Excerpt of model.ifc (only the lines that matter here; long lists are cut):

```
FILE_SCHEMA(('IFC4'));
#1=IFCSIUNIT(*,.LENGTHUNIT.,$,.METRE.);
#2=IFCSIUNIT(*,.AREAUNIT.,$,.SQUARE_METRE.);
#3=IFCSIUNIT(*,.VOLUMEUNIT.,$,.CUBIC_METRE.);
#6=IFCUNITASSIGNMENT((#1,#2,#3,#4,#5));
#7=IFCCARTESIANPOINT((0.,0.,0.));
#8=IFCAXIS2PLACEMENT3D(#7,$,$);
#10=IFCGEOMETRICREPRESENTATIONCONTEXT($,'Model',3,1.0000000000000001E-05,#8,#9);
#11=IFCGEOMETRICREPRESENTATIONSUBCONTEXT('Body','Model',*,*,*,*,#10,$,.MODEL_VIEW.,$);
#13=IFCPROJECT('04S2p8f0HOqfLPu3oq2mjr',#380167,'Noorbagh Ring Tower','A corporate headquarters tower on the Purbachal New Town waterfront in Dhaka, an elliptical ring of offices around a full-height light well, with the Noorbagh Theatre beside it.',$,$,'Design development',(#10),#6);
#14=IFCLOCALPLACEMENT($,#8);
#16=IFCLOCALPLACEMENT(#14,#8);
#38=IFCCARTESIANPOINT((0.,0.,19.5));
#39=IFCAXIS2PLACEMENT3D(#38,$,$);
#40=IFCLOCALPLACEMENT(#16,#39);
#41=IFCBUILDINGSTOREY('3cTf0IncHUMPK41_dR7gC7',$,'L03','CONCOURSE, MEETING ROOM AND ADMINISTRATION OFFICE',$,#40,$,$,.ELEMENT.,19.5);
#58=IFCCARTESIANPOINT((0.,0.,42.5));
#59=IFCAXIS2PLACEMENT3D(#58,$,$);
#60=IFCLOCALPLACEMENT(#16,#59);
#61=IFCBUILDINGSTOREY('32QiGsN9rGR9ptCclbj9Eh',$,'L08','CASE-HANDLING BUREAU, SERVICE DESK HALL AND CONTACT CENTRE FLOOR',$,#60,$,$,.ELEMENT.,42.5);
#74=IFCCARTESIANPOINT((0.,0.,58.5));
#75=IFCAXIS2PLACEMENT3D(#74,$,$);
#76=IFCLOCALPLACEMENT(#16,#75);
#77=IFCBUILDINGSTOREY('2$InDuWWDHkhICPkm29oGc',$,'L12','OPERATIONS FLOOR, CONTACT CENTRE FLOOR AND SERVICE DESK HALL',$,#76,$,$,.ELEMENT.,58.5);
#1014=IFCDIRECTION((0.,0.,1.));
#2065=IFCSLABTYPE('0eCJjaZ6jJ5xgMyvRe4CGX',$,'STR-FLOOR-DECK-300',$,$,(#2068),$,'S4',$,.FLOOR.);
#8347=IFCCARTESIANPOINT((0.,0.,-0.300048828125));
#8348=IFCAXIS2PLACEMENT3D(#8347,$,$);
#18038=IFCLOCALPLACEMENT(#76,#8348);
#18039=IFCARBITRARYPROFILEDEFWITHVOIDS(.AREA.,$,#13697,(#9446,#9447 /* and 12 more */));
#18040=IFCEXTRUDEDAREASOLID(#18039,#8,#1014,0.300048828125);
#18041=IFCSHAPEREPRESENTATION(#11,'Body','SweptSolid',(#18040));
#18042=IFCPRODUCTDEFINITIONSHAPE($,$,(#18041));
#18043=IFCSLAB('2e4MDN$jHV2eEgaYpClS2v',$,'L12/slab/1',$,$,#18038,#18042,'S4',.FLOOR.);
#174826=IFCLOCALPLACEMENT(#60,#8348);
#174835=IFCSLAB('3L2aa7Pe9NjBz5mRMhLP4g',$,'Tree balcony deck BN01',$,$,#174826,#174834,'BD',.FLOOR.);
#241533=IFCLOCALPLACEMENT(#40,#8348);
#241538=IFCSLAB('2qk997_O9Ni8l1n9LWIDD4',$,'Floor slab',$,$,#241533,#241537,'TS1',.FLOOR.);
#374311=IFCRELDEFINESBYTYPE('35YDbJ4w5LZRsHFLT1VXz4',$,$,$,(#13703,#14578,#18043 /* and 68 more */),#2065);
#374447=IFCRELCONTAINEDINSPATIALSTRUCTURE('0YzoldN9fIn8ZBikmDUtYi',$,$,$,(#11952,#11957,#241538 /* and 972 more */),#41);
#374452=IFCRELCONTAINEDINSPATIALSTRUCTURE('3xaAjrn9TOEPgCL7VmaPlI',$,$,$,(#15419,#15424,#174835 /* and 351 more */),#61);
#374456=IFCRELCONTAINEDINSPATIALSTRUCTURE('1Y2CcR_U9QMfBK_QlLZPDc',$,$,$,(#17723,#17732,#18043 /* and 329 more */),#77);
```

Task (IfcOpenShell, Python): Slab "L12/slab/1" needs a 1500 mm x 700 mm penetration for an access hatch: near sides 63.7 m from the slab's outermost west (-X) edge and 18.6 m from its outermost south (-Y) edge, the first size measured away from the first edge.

```python
import numpy as np
import ifcopenshell
import ifcopenshell.api.feature
import ifcopenshell.api.geometry
import ifcopenshell.api.root
import ifcopenshell.geom
import ifcopenshell.util.placement
import ifcopenshell.util.representation
import ifcopenshell.util.shape
import ifcopenshell.util.unit

model = ifcopenshell.open("model.ifc")
unit_scale = ifcopenshell.util.unit.calculate_unit_scale(model)
settings = ifcopenshell.geom.settings()


def volume(element):
    """Net volume in cubic metres, openings subtracted."""
    shape = ifcopenshell.geom.create_shape(settings, element)
    return ifcopenshell.util.shape.get_volume(shape.geometry)


slab = model.by_id(18043)
before = volume(slab)

# Extent in the slab's own axes, in metres. The edges named are its -X and -Y sides.
slab_shape = ifcopenshell.geom.create_shape(settings, slab)
vertices = ifcopenshell.util.shape.get_vertices(slab_shape.geometry)
x_min, y_min, bottom = vertices.min(axis=0)
top = vertices[:, 2].max()

opening = ifcopenshell.api.root.create_entity(model, ifc_class="IfcOpeningElement", name="Access hatch opening", predefined_type="OPENING")
context = ifcopenshell.util.representation.get_context(model, "Model", "Body", "MODEL_VIEW")
width, depth = 1.5, 0.7
outline = [(0.0, 0.0), (width, 0.0), (width, depth), (0.0, depth), (0.0, 0.0)]
# Overshoot both faces by 50 mm so the cut is clean.
shape = ifcopenshell.api.geometry.add_slab_representation(
    model, context=context, depth=top - bottom + 0.1, polyline=outline
)
ifcopenshell.api.geometry.assign_representation(model, product=opening, representation=shape)

matrix = ifcopenshell.util.placement.get_local_placement(slab.ObjectPlacement)
matrix[:, 3] = matrix @ np.append(np.array([x_min + 63.7, y_min + 18.6, bottom - 0.05]) / unit_scale, 1.0)
ifcopenshell.api.geometry.edit_object_placement(model, product=opening, matrix=matrix, is_si=False)
ifcopenshell.api.feature.add_feature(model, feature=opening, element=slab)

after = volume(slab)

print(f"slab volume {before:.3f} -> {after:.3f} m3")

model.write("model_rev.ifc")
```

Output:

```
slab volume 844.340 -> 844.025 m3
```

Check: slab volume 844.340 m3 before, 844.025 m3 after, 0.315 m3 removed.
